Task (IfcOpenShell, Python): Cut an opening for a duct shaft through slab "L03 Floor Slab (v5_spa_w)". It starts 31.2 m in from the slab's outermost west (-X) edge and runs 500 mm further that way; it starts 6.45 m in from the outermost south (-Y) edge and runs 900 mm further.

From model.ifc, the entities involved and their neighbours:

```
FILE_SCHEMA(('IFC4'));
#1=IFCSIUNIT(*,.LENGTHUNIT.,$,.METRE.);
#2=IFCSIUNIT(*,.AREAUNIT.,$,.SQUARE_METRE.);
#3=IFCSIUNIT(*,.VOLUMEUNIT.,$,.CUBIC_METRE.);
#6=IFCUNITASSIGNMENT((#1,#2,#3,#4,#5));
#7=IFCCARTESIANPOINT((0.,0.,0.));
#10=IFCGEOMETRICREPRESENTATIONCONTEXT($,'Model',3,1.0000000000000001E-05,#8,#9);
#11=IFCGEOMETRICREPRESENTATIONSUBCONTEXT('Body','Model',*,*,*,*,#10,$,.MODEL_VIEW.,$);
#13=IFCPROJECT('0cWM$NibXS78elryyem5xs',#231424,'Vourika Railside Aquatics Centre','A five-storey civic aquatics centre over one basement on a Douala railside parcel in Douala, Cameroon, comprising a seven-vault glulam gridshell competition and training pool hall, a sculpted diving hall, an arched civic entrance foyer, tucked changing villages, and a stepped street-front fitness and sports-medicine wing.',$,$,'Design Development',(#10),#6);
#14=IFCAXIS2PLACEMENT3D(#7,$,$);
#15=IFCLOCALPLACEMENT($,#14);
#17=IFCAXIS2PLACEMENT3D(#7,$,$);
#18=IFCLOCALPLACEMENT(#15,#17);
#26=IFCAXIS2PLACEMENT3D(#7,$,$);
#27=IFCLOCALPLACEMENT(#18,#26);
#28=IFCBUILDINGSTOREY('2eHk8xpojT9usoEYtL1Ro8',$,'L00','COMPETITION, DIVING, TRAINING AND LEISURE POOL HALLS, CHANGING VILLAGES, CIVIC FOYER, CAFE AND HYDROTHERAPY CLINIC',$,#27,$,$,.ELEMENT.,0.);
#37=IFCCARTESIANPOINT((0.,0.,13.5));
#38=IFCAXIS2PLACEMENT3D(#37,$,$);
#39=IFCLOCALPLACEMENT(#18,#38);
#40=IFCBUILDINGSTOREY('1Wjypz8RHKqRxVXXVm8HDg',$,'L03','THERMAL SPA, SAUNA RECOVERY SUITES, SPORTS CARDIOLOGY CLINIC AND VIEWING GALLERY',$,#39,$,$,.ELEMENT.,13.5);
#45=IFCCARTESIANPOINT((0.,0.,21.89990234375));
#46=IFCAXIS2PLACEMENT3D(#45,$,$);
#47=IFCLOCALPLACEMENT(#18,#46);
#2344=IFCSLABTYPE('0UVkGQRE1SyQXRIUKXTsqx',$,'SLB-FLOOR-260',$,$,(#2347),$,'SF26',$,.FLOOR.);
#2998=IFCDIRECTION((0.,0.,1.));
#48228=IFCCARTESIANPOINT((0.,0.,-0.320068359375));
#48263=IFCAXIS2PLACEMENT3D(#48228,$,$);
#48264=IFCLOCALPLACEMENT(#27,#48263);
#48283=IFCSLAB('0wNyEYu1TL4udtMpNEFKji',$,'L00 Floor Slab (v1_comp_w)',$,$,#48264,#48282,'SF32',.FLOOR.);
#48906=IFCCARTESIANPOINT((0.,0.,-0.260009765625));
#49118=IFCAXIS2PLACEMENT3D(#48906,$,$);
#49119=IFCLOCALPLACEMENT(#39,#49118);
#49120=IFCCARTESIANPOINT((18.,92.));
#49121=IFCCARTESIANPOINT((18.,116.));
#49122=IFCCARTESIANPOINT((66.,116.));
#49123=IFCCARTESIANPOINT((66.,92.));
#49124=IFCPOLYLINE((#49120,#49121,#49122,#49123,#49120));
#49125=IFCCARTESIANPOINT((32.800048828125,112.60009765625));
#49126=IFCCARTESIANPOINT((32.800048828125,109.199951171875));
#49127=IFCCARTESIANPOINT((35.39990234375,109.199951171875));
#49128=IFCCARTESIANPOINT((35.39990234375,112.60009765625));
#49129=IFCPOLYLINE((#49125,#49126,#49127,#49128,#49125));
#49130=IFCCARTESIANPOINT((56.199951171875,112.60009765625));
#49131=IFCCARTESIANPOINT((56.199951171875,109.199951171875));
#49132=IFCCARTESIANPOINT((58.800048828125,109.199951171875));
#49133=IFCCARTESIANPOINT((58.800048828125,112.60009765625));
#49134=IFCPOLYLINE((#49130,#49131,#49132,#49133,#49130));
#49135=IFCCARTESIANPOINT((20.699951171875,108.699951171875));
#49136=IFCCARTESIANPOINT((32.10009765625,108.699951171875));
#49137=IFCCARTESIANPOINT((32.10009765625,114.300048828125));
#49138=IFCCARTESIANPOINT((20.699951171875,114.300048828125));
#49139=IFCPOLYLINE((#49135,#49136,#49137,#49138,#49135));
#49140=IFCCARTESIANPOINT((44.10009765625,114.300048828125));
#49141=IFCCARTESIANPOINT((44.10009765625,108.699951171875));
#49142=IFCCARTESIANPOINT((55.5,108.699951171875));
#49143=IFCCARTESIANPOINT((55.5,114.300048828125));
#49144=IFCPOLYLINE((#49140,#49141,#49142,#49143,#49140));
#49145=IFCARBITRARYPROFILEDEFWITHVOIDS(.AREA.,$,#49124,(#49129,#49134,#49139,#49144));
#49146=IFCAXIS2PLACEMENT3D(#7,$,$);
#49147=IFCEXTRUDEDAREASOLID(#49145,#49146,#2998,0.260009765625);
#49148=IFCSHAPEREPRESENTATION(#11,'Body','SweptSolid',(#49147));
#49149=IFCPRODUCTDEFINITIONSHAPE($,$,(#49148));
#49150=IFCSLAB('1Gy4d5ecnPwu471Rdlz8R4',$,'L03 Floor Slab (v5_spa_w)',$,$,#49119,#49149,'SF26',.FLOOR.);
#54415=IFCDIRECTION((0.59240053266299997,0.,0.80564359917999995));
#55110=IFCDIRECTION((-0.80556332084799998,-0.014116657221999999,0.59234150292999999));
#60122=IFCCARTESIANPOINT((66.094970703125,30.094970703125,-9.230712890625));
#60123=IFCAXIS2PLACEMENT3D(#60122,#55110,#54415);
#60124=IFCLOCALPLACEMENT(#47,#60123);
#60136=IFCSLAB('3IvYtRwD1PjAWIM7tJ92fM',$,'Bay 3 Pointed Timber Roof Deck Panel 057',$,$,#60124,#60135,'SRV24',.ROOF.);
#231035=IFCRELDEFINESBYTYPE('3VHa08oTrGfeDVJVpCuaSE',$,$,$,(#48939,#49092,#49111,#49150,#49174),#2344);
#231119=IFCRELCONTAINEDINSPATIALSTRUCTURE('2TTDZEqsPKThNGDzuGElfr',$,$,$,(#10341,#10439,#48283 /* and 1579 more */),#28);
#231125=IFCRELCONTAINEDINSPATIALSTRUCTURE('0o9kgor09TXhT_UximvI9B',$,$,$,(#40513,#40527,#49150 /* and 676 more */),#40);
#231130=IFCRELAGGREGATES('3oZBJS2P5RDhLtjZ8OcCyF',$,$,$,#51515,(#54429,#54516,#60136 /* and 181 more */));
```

```python
import numpy as np
import ifcopenshell
import ifcopenshell.api.feature
import ifcopenshell.api.geometry
import ifcopenshell.api.root
import ifcopenshell.geom
import ifcopenshell.util.placement
import ifcopenshell.util.representation
import ifcopenshell.util.shape
import ifcopenshell.util.unit

model = ifcopenshell.open("model.ifc")
unit_scale = ifcopenshell.util.unit.calculate_unit_scale(model)
settings = ifcopenshell.geom.settings()


def volume(element):
    """Net volume in cubic metres, openings subtracted."""
    shape = ifcopenshell.geom.create_shape(settings, element)
    return ifcopenshell.util.shape.get_volume(shape.geometry)


slab = model.by_guid("1Gy4d5ecnPwu471Rdlz8R4")
before = volume(slab)

# Extent in the slab's own axes, in metres. The edges named are its -X and -Y sides.
slab_shape = ifcopenshell.geom.create_shape(settings, slab)
vertices = ifcopenshell.util.shape.get_vertices(slab_shape.geometry)
x_min, y_min, bottom = vertices.min(axis=0)
top = vertices[:, 2].max()

opening = ifcopenshell.api.root.create_entity(model, ifc_class="IfcOpeningElement", name="Duct shaft opening", predefined_type="OPENING")
context = ifcopenshell.util.representation.get_context(model, "Model", "Body", "MODEL_VIEW")
width, depth = 0.5, 0.9
outline = [(0.0, 0.0), (width, 0.0), (width, depth), (0.0, depth), (0.0, 0.0)]
# Overshoot both faces by 50 mm so the cut is clean.
shape = ifcopenshell.api.geometry.add_slab_representation(
    model, context=context, depth=top - bottom + 0.1, polyline=outline
)
ifcopenshell.api.geometry.assign_representation(model, product=opening, representation=shape)

matrix = ifcopenshell.util.placement.get_local_placement(slab.ObjectPlacement)
matrix[:, 3] = matrix @ np.append(np.array([x_min + 31.2, y_min + 6.45, bottom - 0.05]) / unit_scale, 1.0)
ifcopenshell.api.geometry.edit_object_placement(model, product=opening, matrix=matrix, is_si=False)
ifcopenshell.api.feature.add_feature(model, feature=opening, element=slab)

after = volume(slab)

print(f"slab volume {before:.3f} -> {after:.3f} m3")

model.write("model_v2.ifc")
```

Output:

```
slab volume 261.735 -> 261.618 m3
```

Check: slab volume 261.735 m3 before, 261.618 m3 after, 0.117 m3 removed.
